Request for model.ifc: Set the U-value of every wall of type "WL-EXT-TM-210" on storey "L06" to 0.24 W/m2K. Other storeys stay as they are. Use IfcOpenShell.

First a look at what the model holds.

```python
import ifcopenshell
import ifcopenshell.util.element

model = ifcopenshell.open("model.ifc")
print(model.schema)
storey = next(s for s in model.by_type("IfcBuildingStorey") if s.Name == "L06")
walls = [e for e in ifcopenshell.util.element.get_decomposition(storey) if e.is_a("IfcWall")]
seen = {}
for e in walls:
    element_type = ifcopenshell.util.element.get_type(e)
    key = (element_type.Name if element_type != e and element_type else None, ifcopenshell.util.element.get_pset(e, "Pset_WallCommon", "ThermalTransmittance"))
    seen[key] = seen.get(key, 0) + 1
for (name, value), count in sorted(seen.items(), key=str):
    print(count, "x", name, "|", value)
```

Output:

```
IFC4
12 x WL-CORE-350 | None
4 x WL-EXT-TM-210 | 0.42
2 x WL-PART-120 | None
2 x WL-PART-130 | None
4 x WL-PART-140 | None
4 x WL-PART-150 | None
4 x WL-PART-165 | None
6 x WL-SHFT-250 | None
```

```python
import ifcopenshell
import ifcopenshell.api.pset
import ifcopenshell.util.element

model = ifcopenshell.open("model.ifc")

storey = next(s for s in model.by_type("IfcBuildingStorey") if s.Name == "L06")
walls = [e for e in ifcopenshell.util.element.get_decomposition(storey) if e.is_a("IfcWall")]

count = 0
for e in walls:
    element_type = ifcopenshell.util.element.get_type(e)
    if element_type in (None, e) or element_type.Name != "WL-EXT-TM-210":
        continue
    # add_pset returns the element's existing set when there is one.
    pset = ifcopenshell.api.pset.add_pset(model, product=e, name="Pset_WallCommon")
    ifcopenshell.api.pset.edit_pset(model, pset=pset, properties={"ThermalTransmittance": 0.24})
    count += 1

print(count, "walls updated")

model.write("model_v2.ifc")
```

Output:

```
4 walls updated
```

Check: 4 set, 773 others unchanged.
